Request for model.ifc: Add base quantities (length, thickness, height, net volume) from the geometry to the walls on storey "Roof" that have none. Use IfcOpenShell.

First a look at what the model holds.

```python
import ifcopenshell
import ifcopenshell.util.element
import ifcopenshell.util.unit

model = ifcopenshell.open("model.ifc")
print(model.schema)
for unit_type in ("LENGTHUNIT", "AREAUNIT", "VOLUMEUNIT"):
    print(unit_type, ifcopenshell.util.unit.calculate_unit_scale(model, unit_type))
storey = next(s for s in model.by_type("IfcBuildingStorey") if s.Name == "Roof")
walls = [e for e in ifcopenshell.util.element.get_decomposition(storey) if e.is_a("IfcWall")]
for e in sorted(walls, key=lambda e: e.id()):
    print(e.id(), e.is_a(), e.Name, list(ifcopenshell.util.element.get_psets(e, qtos_only=True)), sep=" | ")
```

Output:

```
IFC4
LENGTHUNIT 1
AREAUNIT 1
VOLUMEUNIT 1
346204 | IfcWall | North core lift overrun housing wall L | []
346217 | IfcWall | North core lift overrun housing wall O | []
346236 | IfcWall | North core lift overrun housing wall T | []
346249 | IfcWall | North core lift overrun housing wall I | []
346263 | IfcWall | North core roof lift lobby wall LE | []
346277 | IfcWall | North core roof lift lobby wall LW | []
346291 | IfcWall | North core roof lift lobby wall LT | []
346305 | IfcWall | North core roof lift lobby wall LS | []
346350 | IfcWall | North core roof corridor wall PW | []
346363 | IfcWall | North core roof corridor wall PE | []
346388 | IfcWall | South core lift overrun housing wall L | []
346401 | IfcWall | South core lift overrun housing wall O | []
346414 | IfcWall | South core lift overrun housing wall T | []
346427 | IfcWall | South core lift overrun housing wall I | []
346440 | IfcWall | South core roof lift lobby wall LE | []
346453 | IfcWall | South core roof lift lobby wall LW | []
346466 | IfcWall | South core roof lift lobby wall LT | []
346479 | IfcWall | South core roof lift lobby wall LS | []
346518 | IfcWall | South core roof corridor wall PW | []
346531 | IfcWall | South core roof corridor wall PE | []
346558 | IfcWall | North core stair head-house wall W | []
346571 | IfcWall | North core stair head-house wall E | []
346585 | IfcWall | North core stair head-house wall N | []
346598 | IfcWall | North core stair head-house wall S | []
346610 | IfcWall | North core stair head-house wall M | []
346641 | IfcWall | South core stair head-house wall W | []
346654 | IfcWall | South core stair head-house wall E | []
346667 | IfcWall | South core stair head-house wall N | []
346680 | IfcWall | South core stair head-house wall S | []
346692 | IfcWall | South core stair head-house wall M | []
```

```python
import ifcopenshell
import ifcopenshell.api.pset
import ifcopenshell.geom
import ifcopenshell.util.element
import ifcopenshell.util.shape
import ifcopenshell.util.unit

model = ifcopenshell.open("model.ifc")
unit_scale = ifcopenshell.util.unit.calculate_unit_scale(model)
volume_scale = ifcopenshell.util.unit.calculate_unit_scale(model, "VOLUMEUNIT")
settings = ifcopenshell.geom.settings()

storey = next(s for s in model.by_type("IfcBuildingStorey") if s.Name == "Roof")
walls = [e for e in ifcopenshell.util.element.get_decomposition(storey) if e.is_a("IfcWall")]

for e in sorted(walls, key=lambda e: e.id()):
    if ifcopenshell.util.element.get_psets(e, qtos_only=True, should_inherit=False):
        continue
    # Geometry comes back in metres, in the element's own axes.
    shape = ifcopenshell.geom.create_shape(settings, e)
    values = {
        "Length": ifcopenshell.util.shape.get_x(shape.geometry) / unit_scale,
        "Width": ifcopenshell.util.shape.get_y(shape.geometry) / unit_scale,
        "Height": ifcopenshell.util.shape.get_z(shape.geometry) / unit_scale,
        "NetVolume": ifcopenshell.util.shape.get_volume(shape.geometry) / volume_scale,
    }
    qto = ifcopenshell.api.pset.add_qto(model, product=e, name="Qto_WallBaseQuantities")
    ifcopenshell.api.pset.edit_qto(model, qto=qto, properties=values)
    print(e.id(), {k: round(v, 3) for k, v in values.items()})

model.write("model_updated.ifc")
```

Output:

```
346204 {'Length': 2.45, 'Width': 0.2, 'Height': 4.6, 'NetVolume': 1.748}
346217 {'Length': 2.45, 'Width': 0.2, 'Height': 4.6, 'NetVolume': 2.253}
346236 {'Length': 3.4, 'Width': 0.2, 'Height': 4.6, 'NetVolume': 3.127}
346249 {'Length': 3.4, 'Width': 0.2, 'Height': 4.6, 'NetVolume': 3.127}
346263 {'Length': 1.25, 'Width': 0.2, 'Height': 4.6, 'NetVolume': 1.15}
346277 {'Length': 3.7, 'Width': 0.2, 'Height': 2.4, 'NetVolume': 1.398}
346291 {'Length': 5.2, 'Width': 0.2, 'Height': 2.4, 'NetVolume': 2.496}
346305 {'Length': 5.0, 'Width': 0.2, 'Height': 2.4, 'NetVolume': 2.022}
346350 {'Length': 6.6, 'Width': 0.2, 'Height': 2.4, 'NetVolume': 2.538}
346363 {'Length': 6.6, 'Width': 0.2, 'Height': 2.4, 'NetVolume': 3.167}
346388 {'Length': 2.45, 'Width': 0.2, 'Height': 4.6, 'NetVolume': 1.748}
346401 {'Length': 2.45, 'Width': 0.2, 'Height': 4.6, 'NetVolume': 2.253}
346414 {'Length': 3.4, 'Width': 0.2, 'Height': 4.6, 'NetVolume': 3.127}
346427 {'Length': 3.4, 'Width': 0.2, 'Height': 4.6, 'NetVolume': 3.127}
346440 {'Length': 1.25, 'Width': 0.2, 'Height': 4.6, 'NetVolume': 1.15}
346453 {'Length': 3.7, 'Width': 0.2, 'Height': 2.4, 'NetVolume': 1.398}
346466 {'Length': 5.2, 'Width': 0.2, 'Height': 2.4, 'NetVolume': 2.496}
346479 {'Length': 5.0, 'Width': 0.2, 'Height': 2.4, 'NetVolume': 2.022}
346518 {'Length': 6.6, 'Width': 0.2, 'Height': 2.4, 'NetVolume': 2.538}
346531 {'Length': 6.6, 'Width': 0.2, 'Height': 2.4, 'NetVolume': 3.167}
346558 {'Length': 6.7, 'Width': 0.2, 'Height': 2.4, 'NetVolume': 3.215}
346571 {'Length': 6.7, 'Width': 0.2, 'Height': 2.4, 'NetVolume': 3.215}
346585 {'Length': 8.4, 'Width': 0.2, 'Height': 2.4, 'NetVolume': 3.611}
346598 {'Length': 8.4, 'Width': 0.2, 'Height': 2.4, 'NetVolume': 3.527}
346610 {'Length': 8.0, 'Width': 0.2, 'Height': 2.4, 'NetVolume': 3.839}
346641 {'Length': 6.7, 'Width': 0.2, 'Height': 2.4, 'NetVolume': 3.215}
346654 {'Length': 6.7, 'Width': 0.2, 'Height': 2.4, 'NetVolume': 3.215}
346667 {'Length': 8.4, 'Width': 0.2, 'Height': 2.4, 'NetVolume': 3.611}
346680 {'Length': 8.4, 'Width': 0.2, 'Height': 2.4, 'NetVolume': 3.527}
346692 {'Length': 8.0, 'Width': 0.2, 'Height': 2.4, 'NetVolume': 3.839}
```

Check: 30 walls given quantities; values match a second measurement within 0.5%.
